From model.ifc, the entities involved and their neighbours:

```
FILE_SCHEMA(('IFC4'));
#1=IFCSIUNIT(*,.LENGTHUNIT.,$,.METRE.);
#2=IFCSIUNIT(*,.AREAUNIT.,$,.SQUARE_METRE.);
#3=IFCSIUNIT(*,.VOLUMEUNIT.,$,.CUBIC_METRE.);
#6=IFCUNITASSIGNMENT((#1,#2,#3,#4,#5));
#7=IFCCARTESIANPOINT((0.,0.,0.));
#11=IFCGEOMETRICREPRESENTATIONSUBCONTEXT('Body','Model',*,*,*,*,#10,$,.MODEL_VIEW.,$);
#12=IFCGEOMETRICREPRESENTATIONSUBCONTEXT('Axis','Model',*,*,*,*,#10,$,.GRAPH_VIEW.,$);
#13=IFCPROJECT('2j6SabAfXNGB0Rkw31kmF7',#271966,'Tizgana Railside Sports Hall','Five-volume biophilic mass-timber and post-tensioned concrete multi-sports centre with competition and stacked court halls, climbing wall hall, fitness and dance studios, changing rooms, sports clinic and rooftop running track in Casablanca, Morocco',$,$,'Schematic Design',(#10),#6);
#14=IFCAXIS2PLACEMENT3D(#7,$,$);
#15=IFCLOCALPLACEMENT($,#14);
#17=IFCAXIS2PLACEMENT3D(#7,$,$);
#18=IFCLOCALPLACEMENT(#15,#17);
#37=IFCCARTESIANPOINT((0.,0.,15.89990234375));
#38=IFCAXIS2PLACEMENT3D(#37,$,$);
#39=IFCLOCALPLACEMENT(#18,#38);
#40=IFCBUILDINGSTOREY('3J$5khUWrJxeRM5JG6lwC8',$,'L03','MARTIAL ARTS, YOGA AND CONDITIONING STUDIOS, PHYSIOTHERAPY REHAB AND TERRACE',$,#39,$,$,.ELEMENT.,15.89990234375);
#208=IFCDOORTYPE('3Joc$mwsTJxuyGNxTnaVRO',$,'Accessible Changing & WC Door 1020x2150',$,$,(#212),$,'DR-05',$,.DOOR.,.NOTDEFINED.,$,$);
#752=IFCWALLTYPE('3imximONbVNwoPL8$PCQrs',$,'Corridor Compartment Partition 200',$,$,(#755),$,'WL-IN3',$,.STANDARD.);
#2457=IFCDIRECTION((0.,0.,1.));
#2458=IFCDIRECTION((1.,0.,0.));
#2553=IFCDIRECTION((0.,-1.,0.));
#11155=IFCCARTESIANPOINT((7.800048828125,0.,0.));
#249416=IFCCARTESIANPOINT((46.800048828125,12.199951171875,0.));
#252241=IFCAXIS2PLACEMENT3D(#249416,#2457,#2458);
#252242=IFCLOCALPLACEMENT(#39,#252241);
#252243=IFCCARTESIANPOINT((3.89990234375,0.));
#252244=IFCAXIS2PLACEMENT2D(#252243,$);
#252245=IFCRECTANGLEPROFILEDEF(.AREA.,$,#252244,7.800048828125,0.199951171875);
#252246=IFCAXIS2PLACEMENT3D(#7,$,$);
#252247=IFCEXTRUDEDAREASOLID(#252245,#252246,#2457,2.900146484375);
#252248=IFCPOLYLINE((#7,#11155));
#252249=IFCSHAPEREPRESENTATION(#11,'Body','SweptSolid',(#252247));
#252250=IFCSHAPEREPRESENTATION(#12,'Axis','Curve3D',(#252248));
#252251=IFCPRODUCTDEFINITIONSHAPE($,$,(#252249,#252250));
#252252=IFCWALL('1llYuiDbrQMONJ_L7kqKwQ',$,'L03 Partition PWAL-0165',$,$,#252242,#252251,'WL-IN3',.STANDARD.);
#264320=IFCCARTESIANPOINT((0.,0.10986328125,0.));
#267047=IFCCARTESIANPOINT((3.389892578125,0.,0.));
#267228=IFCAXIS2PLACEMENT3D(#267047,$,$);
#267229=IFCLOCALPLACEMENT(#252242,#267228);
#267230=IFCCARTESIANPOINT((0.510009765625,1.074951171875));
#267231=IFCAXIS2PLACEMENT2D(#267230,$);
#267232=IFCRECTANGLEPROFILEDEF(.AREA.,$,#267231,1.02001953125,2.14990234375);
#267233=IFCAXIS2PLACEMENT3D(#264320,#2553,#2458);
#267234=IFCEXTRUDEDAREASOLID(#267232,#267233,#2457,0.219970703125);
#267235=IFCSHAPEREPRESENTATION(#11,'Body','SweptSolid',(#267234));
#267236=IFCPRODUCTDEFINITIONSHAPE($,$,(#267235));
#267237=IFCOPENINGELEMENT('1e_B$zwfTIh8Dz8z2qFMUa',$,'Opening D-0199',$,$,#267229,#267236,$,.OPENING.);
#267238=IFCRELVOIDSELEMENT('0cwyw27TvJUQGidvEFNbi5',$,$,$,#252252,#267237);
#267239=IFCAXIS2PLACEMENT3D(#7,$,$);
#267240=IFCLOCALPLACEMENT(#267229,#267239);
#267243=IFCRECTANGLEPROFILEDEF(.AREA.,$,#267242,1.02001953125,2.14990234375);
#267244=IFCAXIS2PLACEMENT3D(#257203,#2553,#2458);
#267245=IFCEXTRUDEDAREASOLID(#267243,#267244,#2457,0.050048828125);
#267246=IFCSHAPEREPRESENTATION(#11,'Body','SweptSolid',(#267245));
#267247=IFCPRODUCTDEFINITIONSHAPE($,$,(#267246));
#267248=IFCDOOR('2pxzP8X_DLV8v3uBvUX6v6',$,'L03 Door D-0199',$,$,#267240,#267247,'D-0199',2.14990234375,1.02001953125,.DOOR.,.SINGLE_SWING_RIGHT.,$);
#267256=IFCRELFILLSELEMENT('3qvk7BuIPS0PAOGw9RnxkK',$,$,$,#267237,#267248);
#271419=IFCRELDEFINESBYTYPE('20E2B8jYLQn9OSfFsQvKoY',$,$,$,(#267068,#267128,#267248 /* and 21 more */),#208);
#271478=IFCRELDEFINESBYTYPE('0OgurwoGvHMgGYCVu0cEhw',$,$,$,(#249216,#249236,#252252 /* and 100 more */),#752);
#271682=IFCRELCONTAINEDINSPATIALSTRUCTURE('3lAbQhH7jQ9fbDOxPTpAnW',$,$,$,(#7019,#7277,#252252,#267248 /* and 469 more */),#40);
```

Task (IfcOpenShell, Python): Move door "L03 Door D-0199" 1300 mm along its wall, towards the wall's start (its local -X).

```python
import ifcopenshell
import ifcopenshell.api.geometry
import ifcopenshell.util.placement
import ifcopenshell.util.unit

model = ifcopenshell.open("model.ifc")
unit_scale = ifcopenshell.util.unit.calculate_unit_scale(model)

door = model.by_guid("2pxzP8X_DLV8v3uBvUX6v6")
opening = door.FillsVoids[0].RelatingOpeningElement
wall = opening.VoidsElements[0].RelatingBuildingElement

wall_matrix = ifcopenshell.util.placement.get_local_placement(wall.ObjectPlacement)
shift = wall_matrix[:3, 0] * -1.3 / unit_scale
before = ifcopenshell.util.placement.get_local_placement(door.ObjectPlacement)[:3, 3].copy()

# The door is placed relative to its opening, so it follows when the opening moves.
matrix = ifcopenshell.util.placement.get_local_placement(opening.ObjectPlacement)
matrix[:3, 3] += shift
ifcopenshell.api.geometry.edit_object_placement(
    model, product=opening, matrix=matrix, is_si=False, should_transform_children=True
)

after = ifcopenshell.util.placement.get_local_placement(door.ObjectPlacement)[:3, 3]
print("door moved by", (after - before).round(3) + 0.0)

model.write("model_rev.ifc")
```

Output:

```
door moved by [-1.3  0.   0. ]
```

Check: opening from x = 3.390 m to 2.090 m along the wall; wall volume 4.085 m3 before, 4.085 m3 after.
